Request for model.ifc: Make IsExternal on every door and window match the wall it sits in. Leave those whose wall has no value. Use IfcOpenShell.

First a look at what the model holds.

```python
import ifcopenshell
import ifcopenshell.util.element

model = ifcopenshell.open("model.ifc")
print(model.schema)
seen = {}
for e in model.by_type("IfcDoor") + model.by_type("IfcWindow"):
    if not e.FillsVoids:
        continue
    host = e.FillsVoids[0].RelatingOpeningElement.VoidsElements[0].RelatingBuildingElement
    own = ifcopenshell.util.element.get_pset(e, f"Pset_{e.is_a()[3:].removesuffix('StandardCase')}Common", "IsExternal")
    wall = ifcopenshell.util.element.get_pset(host, "Pset_WallCommon", "IsExternal")
    seen[e.is_a(), own, wall] = seen.get((e.is_a(), own, wall), 0) + 1
for (cls, own, wall), count in sorted(seen.items(), key=str):
    print(count, cls, "IsExternal:", own, "| host wall:", wall)
```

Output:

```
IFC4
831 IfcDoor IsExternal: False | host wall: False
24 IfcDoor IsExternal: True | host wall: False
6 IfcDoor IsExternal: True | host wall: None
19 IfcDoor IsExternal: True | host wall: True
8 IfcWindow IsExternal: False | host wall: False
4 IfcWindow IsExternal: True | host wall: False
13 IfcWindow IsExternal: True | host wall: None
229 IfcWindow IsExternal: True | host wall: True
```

```python
import ifcopenshell
import ifcopenshell.api.pset
import ifcopenshell.util.element

model = ifcopenshell.open("model.ifc")

count = 0
for ifc_class, pset_name in (("IfcDoor", "Pset_DoorCommon"), ("IfcWindow", "Pset_WindowCommon")):
    for e in model.by_type(ifc_class):
        if not e.FillsVoids:
            continue
        host = e.FillsVoids[0].RelatingOpeningElement.VoidsElements[0].RelatingBuildingElement
        external = ifcopenshell.util.element.get_pset(host, "Pset_WallCommon", "IsExternal")
        if external is None or ifcopenshell.util.element.get_pset(e, pset_name, "IsExternal") == external:
            continue
        pset = ifcopenshell.api.pset.add_pset(model, product=e, name=pset_name)
        ifcopenshell.api.pset.edit_pset(model, pset=pset, properties={"IsExternal": external})
        count += 1

print(count, "updated")

model.write("model-out.ifc")
```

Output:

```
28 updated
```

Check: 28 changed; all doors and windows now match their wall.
